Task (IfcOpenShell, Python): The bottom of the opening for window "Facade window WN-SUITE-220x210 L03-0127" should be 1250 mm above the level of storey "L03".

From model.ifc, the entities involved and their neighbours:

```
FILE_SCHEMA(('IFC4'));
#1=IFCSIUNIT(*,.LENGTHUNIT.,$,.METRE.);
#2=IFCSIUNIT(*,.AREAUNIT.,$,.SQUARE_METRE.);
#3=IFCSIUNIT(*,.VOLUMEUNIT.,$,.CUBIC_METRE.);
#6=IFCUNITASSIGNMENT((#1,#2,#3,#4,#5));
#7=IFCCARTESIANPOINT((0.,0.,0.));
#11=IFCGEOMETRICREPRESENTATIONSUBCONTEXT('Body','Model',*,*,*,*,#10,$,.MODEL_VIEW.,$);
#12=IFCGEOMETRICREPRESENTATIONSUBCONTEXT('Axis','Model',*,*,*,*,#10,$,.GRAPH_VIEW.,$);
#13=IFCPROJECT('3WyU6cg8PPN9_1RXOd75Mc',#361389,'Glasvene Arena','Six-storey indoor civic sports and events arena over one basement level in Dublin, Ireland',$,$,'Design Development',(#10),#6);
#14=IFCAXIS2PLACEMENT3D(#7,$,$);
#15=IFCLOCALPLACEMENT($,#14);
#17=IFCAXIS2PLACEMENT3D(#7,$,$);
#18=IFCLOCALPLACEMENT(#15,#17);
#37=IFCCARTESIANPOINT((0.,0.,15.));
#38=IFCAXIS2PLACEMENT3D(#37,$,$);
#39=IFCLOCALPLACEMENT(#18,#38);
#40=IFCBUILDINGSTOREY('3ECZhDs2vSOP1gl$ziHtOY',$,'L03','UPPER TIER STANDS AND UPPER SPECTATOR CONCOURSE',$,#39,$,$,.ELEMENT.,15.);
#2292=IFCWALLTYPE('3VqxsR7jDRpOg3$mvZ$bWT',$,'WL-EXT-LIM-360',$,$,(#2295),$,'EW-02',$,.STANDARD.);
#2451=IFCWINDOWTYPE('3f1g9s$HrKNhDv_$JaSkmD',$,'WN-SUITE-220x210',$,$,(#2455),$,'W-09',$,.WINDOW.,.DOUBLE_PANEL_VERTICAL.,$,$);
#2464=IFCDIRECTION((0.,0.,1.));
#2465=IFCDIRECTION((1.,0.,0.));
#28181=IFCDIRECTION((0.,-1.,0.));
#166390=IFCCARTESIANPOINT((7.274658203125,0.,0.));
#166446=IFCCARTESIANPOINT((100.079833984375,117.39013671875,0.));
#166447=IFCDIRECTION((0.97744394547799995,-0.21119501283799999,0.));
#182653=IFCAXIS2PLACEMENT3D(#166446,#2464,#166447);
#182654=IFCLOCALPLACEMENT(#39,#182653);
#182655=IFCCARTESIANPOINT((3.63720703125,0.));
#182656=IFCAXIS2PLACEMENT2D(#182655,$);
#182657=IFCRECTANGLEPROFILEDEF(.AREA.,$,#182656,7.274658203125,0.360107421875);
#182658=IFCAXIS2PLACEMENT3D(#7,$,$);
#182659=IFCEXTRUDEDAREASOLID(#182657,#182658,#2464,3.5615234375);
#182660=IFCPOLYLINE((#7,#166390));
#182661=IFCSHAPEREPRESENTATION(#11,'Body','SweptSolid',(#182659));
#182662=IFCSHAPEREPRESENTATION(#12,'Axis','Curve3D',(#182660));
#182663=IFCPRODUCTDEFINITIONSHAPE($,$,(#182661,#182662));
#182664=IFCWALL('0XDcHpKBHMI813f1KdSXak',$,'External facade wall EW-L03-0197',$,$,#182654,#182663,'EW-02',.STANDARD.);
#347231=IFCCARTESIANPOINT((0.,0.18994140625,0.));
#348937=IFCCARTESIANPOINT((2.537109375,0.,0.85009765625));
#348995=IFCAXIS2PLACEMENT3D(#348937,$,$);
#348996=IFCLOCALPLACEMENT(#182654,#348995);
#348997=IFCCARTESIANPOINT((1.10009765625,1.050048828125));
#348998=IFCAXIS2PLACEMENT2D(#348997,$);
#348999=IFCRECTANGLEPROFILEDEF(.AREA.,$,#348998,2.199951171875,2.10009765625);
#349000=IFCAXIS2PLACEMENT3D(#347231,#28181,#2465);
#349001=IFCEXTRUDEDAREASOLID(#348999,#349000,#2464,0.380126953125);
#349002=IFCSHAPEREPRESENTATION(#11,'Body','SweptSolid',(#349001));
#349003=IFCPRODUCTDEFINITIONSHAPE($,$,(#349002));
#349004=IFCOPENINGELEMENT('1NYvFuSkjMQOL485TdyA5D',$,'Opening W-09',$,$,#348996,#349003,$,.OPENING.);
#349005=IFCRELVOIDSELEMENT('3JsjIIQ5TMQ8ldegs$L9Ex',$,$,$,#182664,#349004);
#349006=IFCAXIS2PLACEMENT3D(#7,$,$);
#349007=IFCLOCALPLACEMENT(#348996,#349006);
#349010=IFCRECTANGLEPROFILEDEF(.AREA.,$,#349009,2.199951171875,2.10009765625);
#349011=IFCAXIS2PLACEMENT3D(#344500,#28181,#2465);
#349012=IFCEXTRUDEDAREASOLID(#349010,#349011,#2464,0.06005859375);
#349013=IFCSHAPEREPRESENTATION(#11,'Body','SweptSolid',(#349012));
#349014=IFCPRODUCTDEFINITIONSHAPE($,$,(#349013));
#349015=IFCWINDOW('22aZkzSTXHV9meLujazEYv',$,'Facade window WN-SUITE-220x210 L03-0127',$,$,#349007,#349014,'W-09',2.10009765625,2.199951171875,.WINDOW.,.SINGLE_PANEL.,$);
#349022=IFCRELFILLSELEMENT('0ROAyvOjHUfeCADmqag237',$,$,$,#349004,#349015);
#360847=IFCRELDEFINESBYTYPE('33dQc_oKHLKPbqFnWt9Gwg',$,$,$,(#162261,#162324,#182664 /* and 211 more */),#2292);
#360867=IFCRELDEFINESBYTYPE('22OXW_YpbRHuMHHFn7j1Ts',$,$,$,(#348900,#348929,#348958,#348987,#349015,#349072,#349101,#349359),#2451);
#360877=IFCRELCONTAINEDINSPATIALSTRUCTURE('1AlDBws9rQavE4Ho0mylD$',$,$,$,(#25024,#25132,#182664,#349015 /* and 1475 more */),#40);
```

```python
import numpy as np
import ifcopenshell
import ifcopenshell.api.geometry
import ifcopenshell.geom
import ifcopenshell.util.element
import ifcopenshell.util.placement
import ifcopenshell.util.shape
import ifcopenshell.util.unit

model = ifcopenshell.open("model.ifc")
unit_scale = ifcopenshell.util.unit.calculate_unit_scale(model)

window = model.by_guid("22aZkzSTXHV9meLujazEYv")
opening = window.FillsVoids[0].RelatingOpeningElement
storey = ifcopenshell.util.element.get_container(window, ifc_class="IfcBuildingStorey")
level = ifcopenshell.util.placement.get_local_placement(storey.ObjectPlacement)[2, 3]

# The opening's origin need not be at the sill, so measure its lowest point.
shape = ifcopenshell.geom.create_shape(ifcopenshell.geom.settings(), opening)
bottom = ifcopenshell.util.shape.get_shape_bottom_elevation(shape, shape.geometry) / unit_scale
dz = level + 1.25 - bottom

shift = np.array([0.0, 0.0, dz])
# The window is placed relative to its opening, so it follows when the opening moves.
matrix = ifcopenshell.util.placement.get_local_placement(opening.ObjectPlacement)
matrix[:3, 3] += shift
ifcopenshell.api.geometry.edit_object_placement(
    model, product=opening, matrix=matrix, is_si=False, should_transform_children=True
)

print(f"moved by {dz * unit_scale:+.3f} m")

model.write("model_v2.ifc")
```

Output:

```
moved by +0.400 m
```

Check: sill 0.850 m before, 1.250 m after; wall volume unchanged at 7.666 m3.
